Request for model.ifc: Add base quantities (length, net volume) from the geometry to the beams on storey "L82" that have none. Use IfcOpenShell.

First a look at what the model holds.

```python
import ifcopenshell
import ifcopenshell.util.element
import ifcopenshell.util.unit

model = ifcopenshell.open("model.ifc")
print(model.schema)
for unit_type in ("LENGTHUNIT", "AREAUNIT", "VOLUMEUNIT"):
    print(unit_type, ifcopenshell.util.unit.calculate_unit_scale(model, unit_type))
storey = next(s for s in model.by_type("IfcBuildingStorey") if s.Name == "L82")
beams = [e for e in ifcopenshell.util.element.get_decomposition(storey) if e.is_a("IfcBeam")]
for e in sorted(beams, key=lambda e: e.id()):
    print(e.id(), e.is_a(), e.Name, list(ifcopenshell.util.element.get_psets(e, qtos_only=True)), sep=" | ")
```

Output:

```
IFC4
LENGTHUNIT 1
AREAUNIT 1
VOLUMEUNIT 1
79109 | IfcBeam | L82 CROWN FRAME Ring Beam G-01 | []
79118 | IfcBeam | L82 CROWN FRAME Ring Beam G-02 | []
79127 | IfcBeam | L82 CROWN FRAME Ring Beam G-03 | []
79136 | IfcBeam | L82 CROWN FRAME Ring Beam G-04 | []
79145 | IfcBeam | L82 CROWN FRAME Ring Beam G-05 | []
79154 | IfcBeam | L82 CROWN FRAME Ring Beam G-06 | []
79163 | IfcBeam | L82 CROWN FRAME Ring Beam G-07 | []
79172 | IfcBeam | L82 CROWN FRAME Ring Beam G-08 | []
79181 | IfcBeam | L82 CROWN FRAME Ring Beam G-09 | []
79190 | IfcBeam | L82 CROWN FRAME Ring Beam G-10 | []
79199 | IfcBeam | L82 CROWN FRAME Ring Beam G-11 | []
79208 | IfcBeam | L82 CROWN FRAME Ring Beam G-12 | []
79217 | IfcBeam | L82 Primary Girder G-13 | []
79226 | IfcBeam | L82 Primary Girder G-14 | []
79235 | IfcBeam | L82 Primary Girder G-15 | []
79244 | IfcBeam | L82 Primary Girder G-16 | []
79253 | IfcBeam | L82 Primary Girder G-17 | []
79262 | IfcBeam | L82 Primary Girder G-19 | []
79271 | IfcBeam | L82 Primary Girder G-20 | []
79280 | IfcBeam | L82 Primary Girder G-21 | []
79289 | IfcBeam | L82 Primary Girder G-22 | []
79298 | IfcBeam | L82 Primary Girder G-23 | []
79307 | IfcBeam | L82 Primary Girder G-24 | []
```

```python
import ifcopenshell
import ifcopenshell.api.pset
import ifcopenshell.geom
import ifcopenshell.util.element
import ifcopenshell.util.shape
import ifcopenshell.util.unit

model = ifcopenshell.open("model.ifc")
unit_scale = ifcopenshell.util.unit.calculate_unit_scale(model)
volume_scale = ifcopenshell.util.unit.calculate_unit_scale(model, "VOLUMEUNIT")
settings = ifcopenshell.geom.settings()

storey = next(s for s in model.by_type("IfcBuildingStorey") if s.Name == "L82")
beams = [e for e in ifcopenshell.util.element.get_decomposition(storey) if e.is_a("IfcBeam")]

for e in sorted(beams, key=lambda e: e.id()):
    if ifcopenshell.util.element.get_psets(e, qtos_only=True, should_inherit=False):
        continue
    # Geometry comes back in metres, in the element's own axes.
    shape = ifcopenshell.geom.create_shape(settings, e)
    values = {
        "Length": ifcopenshell.util.shape.get_max_xyz(shape.geometry) / unit_scale,
        "NetVolume": ifcopenshell.util.shape.get_volume(shape.geometry) / volume_scale,
    }
    qto = ifcopenshell.api.pset.add_qto(model, product=e, name="Qto_BeamBaseQuantities")
    ifcopenshell.api.pset.edit_qto(model, qto=qto, properties=values)
    print(e.id(), {k: round(v, 3) for k, v in values.items()})

model.write("model_rev.ifc")
```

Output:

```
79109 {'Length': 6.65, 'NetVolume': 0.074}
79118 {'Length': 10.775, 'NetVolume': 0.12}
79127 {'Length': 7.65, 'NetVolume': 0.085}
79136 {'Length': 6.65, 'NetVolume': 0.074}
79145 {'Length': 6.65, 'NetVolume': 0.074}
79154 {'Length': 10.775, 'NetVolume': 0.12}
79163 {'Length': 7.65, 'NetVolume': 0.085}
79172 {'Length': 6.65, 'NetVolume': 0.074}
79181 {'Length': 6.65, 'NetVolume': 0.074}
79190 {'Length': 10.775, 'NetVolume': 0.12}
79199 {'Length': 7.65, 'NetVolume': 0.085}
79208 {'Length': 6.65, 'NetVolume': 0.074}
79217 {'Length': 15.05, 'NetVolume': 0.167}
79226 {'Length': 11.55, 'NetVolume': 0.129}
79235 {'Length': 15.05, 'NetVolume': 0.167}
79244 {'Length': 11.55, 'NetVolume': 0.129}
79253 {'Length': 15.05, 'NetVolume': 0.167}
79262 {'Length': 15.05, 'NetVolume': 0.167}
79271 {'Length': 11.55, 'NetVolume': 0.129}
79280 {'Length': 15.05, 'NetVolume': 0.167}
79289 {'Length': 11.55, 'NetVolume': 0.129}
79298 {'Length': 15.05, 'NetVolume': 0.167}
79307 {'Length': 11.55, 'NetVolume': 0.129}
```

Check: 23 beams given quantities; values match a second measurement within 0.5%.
